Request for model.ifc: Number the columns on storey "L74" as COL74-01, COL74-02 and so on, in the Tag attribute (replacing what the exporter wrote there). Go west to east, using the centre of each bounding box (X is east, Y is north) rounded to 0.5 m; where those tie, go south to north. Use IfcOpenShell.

First a look at what the model holds.

```python
import ifcopenshell
import ifcopenshell.util.element
import ifcopenshell.util.placement

model = ifcopenshell.open("model.ifc")
print(model.schema)
storey = next(s for s in model.by_type("IfcBuildingStorey") if s.Name == "L74")
columns = [e for e in ifcopenshell.util.element.get_decomposition(storey) if e.is_a("IfcColumn")]
for e in sorted(columns, key=lambda e: e.id()):
    origin = ifcopenshell.util.placement.get_local_placement(e.ObjectPlacement)[:3, 3]
    print(e.id(), e.Tag, e.Name, origin.round(2) + 0.0, sep=" | ")
```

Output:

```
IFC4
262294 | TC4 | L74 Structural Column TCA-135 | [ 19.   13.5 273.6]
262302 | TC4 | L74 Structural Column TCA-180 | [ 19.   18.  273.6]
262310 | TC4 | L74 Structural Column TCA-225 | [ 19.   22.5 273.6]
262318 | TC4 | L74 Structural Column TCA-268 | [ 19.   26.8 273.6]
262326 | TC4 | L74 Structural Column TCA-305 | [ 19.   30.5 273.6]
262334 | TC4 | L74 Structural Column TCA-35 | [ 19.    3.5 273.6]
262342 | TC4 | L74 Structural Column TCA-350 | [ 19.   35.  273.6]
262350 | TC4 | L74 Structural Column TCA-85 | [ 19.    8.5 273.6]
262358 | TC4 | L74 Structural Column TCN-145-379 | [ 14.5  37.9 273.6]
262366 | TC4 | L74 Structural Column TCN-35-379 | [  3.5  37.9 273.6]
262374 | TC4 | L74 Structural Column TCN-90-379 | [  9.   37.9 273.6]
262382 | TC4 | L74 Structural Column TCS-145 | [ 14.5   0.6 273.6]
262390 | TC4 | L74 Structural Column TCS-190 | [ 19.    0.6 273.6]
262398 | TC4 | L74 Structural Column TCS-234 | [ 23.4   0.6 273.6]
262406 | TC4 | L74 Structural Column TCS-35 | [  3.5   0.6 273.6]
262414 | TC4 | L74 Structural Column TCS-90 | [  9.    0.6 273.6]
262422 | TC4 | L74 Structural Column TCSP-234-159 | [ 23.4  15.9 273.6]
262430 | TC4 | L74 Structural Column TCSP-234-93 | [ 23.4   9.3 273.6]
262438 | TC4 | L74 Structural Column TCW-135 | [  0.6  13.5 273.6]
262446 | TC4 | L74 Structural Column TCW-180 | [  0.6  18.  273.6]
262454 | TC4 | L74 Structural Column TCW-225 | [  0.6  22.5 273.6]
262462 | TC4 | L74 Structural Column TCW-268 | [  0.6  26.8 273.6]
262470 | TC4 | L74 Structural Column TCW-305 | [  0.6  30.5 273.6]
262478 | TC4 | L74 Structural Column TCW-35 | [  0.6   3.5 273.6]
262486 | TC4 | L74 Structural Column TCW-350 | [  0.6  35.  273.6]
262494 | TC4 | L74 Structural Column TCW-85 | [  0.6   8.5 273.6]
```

```python
import ifcopenshell
import ifcopenshell.geom
import ifcopenshell.util.element
import ifcopenshell.util.shape

model = ifcopenshell.open("model.ifc")
settings = ifcopenshell.geom.settings()
settings.set("use-world-coords", True)


def centre(element):
    shape = ifcopenshell.geom.create_shape(settings, element)
    return ifcopenshell.util.shape.get_bbox_centroid(shape.geometry)


storey = next(s for s in model.by_type("IfcBuildingStorey") if s.Name == "L74")
columns = [e for e in ifcopenshell.util.element.get_decomposition(storey) if e.is_a("IfcColumn")]

# Insertion points can sit at a corner or the storey origin, so sort by the geometry (in metres).
centres = {e: centre(e) for e in columns}
columns.sort(key=lambda e: (round(centres[e][0] / 0.5), centres[e][1]))

for i, e in enumerate(columns, start=1):
    number = f"COL74-{i:02d}"
    e.Tag = number
    print(e.id(), number)

model.write("model_rev.ifc")
```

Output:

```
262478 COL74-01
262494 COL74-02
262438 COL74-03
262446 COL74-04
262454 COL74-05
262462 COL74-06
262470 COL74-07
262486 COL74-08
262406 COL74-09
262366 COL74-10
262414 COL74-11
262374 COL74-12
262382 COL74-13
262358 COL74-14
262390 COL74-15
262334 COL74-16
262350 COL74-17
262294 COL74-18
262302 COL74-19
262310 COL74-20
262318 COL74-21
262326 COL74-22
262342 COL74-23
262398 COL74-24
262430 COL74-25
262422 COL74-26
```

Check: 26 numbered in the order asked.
